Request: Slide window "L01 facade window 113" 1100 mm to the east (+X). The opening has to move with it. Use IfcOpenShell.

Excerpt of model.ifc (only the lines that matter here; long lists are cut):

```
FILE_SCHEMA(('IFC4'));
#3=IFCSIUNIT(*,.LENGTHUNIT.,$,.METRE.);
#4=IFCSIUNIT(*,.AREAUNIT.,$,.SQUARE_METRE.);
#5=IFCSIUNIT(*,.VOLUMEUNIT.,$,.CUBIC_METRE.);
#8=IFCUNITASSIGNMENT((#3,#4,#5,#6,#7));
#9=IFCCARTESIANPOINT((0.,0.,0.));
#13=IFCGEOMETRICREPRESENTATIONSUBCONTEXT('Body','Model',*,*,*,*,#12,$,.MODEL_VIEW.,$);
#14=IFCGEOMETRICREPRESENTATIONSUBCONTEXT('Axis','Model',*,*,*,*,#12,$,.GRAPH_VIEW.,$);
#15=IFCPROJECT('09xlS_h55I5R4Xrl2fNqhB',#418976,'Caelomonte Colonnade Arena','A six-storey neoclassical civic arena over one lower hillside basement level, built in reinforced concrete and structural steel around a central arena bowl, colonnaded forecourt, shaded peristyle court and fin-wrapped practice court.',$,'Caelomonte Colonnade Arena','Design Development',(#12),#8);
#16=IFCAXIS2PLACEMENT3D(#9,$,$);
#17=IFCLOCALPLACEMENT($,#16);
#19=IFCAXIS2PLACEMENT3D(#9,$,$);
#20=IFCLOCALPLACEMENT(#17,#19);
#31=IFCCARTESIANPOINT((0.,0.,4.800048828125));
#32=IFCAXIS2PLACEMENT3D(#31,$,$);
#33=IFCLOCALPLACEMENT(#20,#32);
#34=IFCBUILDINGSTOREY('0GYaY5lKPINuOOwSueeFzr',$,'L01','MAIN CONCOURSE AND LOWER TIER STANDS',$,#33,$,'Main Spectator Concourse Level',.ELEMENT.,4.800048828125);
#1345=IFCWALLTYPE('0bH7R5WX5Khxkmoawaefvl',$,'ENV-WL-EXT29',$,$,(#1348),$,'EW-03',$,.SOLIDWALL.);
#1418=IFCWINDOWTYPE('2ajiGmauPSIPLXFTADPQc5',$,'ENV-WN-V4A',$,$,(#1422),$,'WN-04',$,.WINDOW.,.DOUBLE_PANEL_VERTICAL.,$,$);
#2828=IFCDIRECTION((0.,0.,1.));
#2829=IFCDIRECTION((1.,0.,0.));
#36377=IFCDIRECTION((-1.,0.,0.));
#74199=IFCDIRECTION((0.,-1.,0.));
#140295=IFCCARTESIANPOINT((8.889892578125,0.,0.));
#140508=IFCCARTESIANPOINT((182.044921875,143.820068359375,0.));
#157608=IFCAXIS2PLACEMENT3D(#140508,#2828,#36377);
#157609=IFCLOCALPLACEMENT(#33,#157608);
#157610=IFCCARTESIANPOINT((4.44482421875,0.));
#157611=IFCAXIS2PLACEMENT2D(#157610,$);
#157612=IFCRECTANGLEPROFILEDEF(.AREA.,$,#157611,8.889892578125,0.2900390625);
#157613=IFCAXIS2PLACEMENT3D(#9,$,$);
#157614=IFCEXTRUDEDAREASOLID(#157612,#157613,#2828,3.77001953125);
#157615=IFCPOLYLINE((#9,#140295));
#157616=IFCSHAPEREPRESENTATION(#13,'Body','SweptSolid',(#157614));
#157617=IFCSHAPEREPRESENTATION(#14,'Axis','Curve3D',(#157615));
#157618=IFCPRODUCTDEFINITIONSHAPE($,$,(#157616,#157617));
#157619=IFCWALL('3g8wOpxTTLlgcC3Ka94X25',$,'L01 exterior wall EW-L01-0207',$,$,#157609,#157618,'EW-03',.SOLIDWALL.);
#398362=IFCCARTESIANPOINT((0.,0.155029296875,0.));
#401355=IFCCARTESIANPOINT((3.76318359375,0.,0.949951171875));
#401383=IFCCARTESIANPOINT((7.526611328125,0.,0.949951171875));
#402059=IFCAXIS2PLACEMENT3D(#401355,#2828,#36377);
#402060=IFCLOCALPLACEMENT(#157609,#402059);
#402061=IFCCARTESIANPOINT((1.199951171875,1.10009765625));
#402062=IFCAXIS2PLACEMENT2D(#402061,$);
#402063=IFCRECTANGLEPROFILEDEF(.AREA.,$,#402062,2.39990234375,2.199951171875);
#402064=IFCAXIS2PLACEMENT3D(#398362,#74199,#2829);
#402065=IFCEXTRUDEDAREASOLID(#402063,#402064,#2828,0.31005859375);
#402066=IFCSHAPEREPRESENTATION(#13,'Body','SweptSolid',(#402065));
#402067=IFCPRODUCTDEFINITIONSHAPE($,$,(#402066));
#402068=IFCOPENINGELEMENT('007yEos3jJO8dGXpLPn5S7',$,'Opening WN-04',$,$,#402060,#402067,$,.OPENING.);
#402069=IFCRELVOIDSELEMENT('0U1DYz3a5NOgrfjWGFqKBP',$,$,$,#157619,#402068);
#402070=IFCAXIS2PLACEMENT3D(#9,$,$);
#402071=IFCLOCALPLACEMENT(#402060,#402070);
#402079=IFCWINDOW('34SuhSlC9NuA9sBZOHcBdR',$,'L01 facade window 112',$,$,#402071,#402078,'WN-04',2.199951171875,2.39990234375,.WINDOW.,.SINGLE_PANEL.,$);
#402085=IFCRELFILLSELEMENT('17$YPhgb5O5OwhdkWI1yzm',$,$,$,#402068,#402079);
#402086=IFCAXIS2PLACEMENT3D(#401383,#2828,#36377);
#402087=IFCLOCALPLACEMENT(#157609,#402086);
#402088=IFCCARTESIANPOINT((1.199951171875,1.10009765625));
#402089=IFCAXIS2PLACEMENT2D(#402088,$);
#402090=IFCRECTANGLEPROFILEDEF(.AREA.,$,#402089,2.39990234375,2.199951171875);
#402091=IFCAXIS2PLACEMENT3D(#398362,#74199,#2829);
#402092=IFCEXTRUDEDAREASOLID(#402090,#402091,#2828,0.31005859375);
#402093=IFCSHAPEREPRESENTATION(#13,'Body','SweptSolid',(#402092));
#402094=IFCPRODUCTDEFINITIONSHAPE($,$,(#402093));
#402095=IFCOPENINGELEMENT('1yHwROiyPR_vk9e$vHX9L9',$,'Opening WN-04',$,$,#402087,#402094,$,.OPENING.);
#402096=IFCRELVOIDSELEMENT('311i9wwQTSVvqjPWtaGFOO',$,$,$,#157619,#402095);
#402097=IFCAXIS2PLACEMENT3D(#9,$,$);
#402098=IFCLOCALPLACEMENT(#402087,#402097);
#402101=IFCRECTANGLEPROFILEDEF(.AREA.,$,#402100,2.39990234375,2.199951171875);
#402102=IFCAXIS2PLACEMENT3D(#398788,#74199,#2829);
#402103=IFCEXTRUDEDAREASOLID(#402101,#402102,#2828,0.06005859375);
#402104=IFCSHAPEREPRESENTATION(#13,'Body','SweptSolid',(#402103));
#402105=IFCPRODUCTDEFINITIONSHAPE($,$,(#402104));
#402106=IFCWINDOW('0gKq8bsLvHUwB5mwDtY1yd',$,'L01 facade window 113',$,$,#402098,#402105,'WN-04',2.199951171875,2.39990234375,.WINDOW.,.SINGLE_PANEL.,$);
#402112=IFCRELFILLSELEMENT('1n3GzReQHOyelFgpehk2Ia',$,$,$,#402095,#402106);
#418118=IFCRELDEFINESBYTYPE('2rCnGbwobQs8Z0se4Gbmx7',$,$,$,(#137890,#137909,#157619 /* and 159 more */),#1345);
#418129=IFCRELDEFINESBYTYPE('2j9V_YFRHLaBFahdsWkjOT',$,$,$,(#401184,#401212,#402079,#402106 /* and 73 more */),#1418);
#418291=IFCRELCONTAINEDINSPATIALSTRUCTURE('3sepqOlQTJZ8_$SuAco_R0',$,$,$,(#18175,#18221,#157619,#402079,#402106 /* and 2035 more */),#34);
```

```python
import ifcopenshell
import ifcopenshell.api.geometry
import ifcopenshell.util.placement
import ifcopenshell.util.unit

model = ifcopenshell.open("model.ifc")
unit_scale = ifcopenshell.util.unit.calculate_unit_scale(model)

window = model.by_guid("0gKq8bsLvHUwB5mwDtY1yd")
opening = window.FillsVoids[0].RelatingOpeningElement
wall = opening.VoidsElements[0].RelatingBuildingElement

wall_matrix = ifcopenshell.util.placement.get_local_placement(wall.ObjectPlacement)
shift = wall_matrix[:3, 0] * -1.1 / unit_scale
before = ifcopenshell.util.placement.get_local_placement(window.ObjectPlacement)[:3, 3].copy()

# The window is placed relative to its opening, so it follows when the opening moves.
matrix = ifcopenshell.util.placement.get_local_placement(opening.ObjectPlacement)
matrix[:3, 3] += shift
ifcopenshell.api.geometry.edit_object_placement(
    model, product=opening, matrix=matrix, is_si=False, should_transform_children=True
)

after = ifcopenshell.util.placement.get_local_placement(window.ObjectPlacement)[:3, 3]
print("window moved by", (after - before).round(3) + 0.0)

model.write("model_rev.ifc")
```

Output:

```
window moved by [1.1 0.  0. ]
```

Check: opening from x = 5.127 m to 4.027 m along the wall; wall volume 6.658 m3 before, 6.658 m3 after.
